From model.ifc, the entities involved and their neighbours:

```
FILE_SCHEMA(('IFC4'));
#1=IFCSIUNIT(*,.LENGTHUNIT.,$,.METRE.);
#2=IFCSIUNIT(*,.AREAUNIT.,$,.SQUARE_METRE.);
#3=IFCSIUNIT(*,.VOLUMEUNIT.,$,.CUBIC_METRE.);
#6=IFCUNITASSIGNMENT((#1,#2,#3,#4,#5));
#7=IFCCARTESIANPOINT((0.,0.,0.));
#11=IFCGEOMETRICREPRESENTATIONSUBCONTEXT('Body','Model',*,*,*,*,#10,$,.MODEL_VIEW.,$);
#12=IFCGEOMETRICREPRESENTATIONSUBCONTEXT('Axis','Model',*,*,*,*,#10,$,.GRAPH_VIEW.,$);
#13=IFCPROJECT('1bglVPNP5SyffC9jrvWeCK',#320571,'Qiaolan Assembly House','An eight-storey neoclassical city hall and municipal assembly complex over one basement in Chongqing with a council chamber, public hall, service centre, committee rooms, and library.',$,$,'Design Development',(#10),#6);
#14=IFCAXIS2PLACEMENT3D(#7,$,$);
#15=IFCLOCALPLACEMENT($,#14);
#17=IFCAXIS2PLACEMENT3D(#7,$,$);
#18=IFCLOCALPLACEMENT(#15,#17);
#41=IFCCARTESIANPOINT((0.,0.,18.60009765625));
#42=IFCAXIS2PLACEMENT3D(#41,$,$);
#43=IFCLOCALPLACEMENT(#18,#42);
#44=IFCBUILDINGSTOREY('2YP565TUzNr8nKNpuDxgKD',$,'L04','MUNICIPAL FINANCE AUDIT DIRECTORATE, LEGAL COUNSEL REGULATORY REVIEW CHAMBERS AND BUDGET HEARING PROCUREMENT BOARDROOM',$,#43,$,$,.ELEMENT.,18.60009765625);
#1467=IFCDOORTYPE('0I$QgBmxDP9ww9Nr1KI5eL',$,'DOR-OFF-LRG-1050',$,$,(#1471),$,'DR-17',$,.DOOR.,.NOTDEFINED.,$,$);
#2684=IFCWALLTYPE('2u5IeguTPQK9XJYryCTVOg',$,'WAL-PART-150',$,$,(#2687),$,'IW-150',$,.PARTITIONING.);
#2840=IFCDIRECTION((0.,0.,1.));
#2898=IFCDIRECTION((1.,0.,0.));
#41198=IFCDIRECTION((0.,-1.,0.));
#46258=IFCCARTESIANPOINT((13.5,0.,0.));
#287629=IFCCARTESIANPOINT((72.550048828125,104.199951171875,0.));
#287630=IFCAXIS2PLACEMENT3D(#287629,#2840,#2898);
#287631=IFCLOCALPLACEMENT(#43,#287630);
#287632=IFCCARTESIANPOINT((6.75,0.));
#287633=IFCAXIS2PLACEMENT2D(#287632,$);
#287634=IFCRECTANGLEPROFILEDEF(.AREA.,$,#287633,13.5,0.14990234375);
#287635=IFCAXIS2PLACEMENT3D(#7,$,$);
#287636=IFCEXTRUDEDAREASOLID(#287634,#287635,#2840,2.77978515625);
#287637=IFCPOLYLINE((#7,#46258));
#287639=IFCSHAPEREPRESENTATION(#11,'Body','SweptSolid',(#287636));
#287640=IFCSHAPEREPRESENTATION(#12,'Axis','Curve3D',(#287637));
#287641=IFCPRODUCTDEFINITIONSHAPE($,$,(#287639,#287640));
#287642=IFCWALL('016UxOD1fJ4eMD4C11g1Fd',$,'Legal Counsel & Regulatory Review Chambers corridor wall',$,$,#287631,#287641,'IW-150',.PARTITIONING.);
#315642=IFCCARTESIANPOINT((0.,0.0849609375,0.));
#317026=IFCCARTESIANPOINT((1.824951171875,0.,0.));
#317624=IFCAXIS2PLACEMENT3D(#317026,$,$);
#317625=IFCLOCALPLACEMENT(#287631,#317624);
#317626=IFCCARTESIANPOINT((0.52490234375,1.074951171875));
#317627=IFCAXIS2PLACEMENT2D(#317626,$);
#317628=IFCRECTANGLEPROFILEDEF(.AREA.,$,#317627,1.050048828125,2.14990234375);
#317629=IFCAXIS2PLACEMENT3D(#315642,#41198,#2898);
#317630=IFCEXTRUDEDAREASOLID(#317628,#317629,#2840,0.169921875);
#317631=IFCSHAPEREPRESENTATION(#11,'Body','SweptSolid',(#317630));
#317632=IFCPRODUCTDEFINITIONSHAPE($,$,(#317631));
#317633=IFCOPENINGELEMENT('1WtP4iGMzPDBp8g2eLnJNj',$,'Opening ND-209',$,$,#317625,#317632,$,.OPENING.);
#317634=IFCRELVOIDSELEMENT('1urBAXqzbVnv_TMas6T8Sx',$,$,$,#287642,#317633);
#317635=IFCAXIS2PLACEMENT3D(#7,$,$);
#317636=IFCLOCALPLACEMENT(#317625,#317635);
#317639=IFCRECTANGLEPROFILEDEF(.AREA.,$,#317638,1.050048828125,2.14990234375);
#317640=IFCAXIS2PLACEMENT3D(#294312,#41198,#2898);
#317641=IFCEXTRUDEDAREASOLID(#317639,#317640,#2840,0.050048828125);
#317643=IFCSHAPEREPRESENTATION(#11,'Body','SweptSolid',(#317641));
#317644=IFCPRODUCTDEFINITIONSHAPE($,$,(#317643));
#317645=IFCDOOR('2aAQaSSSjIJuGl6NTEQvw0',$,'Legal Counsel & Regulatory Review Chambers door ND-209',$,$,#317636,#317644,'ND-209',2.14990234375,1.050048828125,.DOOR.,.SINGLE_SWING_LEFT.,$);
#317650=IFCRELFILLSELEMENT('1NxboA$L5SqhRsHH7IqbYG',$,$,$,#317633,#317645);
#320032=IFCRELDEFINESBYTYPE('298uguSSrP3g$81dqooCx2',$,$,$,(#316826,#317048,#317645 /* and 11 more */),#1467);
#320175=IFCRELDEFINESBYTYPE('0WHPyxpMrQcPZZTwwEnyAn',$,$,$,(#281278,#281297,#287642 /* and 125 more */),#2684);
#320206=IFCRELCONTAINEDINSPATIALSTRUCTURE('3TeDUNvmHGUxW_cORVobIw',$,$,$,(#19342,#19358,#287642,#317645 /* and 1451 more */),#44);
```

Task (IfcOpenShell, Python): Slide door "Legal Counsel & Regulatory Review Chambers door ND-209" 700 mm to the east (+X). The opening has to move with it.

```python
import ifcopenshell
import ifcopenshell.api.geometry
import ifcopenshell.util.placement

model = ifcopenshell.open("model.ifc")

door = model.by_id(317645)
opening = door.FillsVoids[0].RelatingOpeningElement
wall = opening.VoidsElements[0].RelatingBuildingElement

wall_matrix = ifcopenshell.util.placement.get_local_placement(wall.ObjectPlacement)
shift = wall_matrix[:3, 0] * 0.7
before = ifcopenshell.util.placement.get_local_placement(door.ObjectPlacement)[:3, 3].copy()

# The door is placed relative to its opening, so it follows when the opening moves.
matrix = ifcopenshell.util.placement.get_local_placement(opening.ObjectPlacement)
matrix[:3, 3] += shift
ifcopenshell.api.geometry.edit_object_placement(
    model, product=opening, matrix=matrix, is_si=False, should_transform_children=True
)

after = ifcopenshell.util.placement.get_local_placement(door.ObjectPlacement)[:3, 3]
print("door moved by", (after - before).round(3) + 0.0)

model.write("model-out.ifc")
```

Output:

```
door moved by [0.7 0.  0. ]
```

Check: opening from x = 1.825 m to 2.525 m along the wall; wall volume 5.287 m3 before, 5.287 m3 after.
